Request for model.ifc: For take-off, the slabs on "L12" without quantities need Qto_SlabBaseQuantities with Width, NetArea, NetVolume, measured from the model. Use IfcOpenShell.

First a look at what the model holds.

```python
import ifcopenshell
import ifcopenshell.util.element
import ifcopenshell.util.unit

model = ifcopenshell.open("model.ifc")
print(model.schema)
for unit_type in ("LENGTHUNIT", "AREAUNIT", "VOLUMEUNIT"):
    print(unit_type, ifcopenshell.util.unit.calculate_unit_scale(model, unit_type))
storey = next(s for s in model.by_type("IfcBuildingStorey") if s.Name == "L12")
slabs = [e for e in ifcopenshell.util.element.get_decomposition(storey) if e.is_a("IfcSlab")]
for e in sorted(slabs, key=lambda e: e.id()):
    print(e.id(), e.is_a(), e.Name, list(ifcopenshell.util.element.get_psets(e, qtos_only=True)), sep=" | ")
```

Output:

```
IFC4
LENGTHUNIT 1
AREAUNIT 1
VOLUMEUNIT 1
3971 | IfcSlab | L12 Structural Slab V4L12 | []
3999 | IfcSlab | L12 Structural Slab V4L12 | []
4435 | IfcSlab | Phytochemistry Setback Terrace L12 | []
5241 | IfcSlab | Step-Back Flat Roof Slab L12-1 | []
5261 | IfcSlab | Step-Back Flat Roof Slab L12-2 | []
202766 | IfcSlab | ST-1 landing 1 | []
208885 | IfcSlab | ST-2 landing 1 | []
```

```python
import ifcopenshell
import ifcopenshell.api.pset
import ifcopenshell.geom
import ifcopenshell.util.element
import ifcopenshell.util.shape
import ifcopenshell.util.unit

model = ifcopenshell.open("model.ifc")
unit_scale = ifcopenshell.util.unit.calculate_unit_scale(model)
area_scale = ifcopenshell.util.unit.calculate_unit_scale(model, "AREAUNIT")
volume_scale = ifcopenshell.util.unit.calculate_unit_scale(model, "VOLUMEUNIT")
settings = ifcopenshell.geom.settings()

storey = next(s for s in model.by_type("IfcBuildingStorey") if s.Name == "L12")
slabs = [e for e in ifcopenshell.util.element.get_decomposition(storey) if e.is_a("IfcSlab")]

for e in sorted(slabs, key=lambda e: e.id()):
    if ifcopenshell.util.element.get_psets(e, qtos_only=True, should_inherit=False):
        continue
    # Geometry comes back in metres, in the element's own axes.
    shape = ifcopenshell.geom.create_shape(settings, e)
    values = {
        "Width": ifcopenshell.util.shape.get_z(shape.geometry) / unit_scale,
        "NetArea": ifcopenshell.util.shape.get_footprint_area(shape.geometry) / area_scale,
        "NetVolume": ifcopenshell.util.shape.get_volume(shape.geometry) / volume_scale,
    }
    qto = ifcopenshell.api.pset.add_qto(model, product=e, name="Qto_SlabBaseQuantities")
    ifcopenshell.api.pset.edit_qto(model, qto=qto, properties=values)
    print(e.id(), {k: round(v, 3) for k, v in values.items()})

model.write("model-out.ifc")
```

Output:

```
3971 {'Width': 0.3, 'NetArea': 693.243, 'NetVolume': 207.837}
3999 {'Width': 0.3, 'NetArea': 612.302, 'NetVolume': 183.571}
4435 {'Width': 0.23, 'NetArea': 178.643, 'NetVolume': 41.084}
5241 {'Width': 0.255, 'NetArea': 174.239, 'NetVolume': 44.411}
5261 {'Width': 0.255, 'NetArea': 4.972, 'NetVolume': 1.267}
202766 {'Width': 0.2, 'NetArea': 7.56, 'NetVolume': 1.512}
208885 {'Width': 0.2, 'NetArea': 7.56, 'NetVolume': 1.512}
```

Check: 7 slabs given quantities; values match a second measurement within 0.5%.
